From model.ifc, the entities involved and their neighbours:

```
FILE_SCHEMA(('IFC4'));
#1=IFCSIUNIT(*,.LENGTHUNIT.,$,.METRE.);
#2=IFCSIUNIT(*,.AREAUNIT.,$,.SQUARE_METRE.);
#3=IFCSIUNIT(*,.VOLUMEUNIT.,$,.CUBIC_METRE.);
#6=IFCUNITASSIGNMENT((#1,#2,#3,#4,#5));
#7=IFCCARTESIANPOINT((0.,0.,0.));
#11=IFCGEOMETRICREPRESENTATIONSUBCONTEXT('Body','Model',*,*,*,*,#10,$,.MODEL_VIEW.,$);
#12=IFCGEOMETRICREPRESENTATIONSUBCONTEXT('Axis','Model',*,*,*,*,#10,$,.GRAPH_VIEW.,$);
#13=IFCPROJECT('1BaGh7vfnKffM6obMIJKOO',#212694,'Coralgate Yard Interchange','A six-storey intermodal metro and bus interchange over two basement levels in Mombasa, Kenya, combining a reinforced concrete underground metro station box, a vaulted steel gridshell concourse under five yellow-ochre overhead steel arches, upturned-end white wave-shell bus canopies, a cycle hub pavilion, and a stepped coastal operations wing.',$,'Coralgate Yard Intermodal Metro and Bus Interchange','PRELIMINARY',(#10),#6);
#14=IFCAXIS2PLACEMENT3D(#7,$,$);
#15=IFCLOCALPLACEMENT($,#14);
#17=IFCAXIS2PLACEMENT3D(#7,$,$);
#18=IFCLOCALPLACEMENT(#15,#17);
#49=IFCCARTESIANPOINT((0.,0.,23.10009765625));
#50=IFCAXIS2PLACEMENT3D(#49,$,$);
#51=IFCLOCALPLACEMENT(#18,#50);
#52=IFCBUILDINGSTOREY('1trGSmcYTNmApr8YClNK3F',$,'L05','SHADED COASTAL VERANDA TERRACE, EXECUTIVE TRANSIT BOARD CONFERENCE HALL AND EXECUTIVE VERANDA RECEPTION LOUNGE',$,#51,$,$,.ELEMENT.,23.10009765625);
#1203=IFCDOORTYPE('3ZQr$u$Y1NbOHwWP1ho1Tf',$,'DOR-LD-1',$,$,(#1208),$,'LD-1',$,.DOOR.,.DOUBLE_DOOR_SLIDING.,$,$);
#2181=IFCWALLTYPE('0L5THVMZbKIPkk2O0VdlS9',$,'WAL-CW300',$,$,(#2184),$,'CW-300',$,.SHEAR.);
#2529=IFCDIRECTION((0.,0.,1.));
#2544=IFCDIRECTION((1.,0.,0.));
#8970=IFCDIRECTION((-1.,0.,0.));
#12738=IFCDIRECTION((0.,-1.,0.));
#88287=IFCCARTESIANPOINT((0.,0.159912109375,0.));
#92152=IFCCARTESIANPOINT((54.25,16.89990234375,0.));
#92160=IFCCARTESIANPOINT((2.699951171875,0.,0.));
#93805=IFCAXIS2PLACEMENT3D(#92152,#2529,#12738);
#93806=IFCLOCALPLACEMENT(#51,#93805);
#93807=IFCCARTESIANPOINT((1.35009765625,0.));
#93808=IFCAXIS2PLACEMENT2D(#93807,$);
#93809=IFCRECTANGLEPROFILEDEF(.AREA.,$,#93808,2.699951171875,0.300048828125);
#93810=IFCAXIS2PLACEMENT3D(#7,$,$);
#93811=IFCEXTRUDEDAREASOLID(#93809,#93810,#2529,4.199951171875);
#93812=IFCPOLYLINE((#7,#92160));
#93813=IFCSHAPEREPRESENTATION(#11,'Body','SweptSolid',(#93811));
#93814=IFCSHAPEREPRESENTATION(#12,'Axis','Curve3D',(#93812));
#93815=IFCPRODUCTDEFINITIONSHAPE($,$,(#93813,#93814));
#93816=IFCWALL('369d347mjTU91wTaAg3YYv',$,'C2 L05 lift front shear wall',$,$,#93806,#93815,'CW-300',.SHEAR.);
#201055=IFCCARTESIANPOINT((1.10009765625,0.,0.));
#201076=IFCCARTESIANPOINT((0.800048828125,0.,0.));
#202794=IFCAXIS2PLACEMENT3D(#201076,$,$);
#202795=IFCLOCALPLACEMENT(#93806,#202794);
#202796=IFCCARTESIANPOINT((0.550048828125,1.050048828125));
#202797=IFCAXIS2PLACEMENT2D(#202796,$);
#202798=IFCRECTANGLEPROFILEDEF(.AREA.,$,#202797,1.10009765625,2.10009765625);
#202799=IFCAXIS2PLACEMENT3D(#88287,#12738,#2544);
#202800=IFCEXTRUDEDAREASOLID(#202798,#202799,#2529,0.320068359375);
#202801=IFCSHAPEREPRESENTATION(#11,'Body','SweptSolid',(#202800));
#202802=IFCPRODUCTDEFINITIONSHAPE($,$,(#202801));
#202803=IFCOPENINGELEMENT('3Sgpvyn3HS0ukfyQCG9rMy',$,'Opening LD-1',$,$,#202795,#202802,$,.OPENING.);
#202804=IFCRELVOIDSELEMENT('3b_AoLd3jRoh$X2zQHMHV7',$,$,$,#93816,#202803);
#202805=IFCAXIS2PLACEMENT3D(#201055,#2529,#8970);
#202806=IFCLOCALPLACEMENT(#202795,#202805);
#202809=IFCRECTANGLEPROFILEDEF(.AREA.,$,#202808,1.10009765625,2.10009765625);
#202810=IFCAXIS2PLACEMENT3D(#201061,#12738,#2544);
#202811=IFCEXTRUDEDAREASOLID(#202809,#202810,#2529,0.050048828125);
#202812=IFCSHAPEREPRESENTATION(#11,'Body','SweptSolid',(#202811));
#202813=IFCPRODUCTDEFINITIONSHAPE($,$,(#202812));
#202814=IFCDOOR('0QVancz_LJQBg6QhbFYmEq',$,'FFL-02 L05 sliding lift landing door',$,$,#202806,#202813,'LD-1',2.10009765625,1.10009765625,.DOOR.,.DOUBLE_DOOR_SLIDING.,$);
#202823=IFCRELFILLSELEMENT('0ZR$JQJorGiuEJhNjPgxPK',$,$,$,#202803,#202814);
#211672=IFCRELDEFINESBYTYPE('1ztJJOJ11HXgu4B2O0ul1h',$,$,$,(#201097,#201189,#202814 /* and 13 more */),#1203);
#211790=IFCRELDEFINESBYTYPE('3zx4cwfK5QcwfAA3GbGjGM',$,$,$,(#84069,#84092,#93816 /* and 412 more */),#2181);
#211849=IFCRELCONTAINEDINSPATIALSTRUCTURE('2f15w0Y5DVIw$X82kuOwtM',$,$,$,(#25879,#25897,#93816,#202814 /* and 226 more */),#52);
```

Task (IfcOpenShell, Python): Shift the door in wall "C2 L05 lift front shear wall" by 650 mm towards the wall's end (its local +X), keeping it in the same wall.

```python
import ifcopenshell
import ifcopenshell.api.geometry
import ifcopenshell.util.placement

model = ifcopenshell.open("model.ifc")

door = model.by_id(202814)
opening = door.FillsVoids[0].RelatingOpeningElement
wall = opening.VoidsElements[0].RelatingBuildingElement

wall_matrix = ifcopenshell.util.placement.get_local_placement(wall.ObjectPlacement)
shift = wall_matrix[:3, 0] * 0.65
before = ifcopenshell.util.placement.get_local_placement(door.ObjectPlacement)[:3, 3].copy()

# The door is placed relative to its opening, so it follows when the opening moves.
matrix = ifcopenshell.util.placement.get_local_placement(opening.ObjectPlacement)
matrix[:3, 3] += shift
ifcopenshell.api.geometry.edit_object_placement(
    model, product=opening, matrix=matrix, is_si=False, should_transform_children=True
)

after = ifcopenshell.util.placement.get_local_placement(door.ObjectPlacement)[:3, 3]
print("door moved by", (after - before).round(3) + 0.0)

model.write("model_rev.ifc")
```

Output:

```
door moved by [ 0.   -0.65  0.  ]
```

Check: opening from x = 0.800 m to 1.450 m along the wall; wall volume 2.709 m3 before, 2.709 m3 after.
